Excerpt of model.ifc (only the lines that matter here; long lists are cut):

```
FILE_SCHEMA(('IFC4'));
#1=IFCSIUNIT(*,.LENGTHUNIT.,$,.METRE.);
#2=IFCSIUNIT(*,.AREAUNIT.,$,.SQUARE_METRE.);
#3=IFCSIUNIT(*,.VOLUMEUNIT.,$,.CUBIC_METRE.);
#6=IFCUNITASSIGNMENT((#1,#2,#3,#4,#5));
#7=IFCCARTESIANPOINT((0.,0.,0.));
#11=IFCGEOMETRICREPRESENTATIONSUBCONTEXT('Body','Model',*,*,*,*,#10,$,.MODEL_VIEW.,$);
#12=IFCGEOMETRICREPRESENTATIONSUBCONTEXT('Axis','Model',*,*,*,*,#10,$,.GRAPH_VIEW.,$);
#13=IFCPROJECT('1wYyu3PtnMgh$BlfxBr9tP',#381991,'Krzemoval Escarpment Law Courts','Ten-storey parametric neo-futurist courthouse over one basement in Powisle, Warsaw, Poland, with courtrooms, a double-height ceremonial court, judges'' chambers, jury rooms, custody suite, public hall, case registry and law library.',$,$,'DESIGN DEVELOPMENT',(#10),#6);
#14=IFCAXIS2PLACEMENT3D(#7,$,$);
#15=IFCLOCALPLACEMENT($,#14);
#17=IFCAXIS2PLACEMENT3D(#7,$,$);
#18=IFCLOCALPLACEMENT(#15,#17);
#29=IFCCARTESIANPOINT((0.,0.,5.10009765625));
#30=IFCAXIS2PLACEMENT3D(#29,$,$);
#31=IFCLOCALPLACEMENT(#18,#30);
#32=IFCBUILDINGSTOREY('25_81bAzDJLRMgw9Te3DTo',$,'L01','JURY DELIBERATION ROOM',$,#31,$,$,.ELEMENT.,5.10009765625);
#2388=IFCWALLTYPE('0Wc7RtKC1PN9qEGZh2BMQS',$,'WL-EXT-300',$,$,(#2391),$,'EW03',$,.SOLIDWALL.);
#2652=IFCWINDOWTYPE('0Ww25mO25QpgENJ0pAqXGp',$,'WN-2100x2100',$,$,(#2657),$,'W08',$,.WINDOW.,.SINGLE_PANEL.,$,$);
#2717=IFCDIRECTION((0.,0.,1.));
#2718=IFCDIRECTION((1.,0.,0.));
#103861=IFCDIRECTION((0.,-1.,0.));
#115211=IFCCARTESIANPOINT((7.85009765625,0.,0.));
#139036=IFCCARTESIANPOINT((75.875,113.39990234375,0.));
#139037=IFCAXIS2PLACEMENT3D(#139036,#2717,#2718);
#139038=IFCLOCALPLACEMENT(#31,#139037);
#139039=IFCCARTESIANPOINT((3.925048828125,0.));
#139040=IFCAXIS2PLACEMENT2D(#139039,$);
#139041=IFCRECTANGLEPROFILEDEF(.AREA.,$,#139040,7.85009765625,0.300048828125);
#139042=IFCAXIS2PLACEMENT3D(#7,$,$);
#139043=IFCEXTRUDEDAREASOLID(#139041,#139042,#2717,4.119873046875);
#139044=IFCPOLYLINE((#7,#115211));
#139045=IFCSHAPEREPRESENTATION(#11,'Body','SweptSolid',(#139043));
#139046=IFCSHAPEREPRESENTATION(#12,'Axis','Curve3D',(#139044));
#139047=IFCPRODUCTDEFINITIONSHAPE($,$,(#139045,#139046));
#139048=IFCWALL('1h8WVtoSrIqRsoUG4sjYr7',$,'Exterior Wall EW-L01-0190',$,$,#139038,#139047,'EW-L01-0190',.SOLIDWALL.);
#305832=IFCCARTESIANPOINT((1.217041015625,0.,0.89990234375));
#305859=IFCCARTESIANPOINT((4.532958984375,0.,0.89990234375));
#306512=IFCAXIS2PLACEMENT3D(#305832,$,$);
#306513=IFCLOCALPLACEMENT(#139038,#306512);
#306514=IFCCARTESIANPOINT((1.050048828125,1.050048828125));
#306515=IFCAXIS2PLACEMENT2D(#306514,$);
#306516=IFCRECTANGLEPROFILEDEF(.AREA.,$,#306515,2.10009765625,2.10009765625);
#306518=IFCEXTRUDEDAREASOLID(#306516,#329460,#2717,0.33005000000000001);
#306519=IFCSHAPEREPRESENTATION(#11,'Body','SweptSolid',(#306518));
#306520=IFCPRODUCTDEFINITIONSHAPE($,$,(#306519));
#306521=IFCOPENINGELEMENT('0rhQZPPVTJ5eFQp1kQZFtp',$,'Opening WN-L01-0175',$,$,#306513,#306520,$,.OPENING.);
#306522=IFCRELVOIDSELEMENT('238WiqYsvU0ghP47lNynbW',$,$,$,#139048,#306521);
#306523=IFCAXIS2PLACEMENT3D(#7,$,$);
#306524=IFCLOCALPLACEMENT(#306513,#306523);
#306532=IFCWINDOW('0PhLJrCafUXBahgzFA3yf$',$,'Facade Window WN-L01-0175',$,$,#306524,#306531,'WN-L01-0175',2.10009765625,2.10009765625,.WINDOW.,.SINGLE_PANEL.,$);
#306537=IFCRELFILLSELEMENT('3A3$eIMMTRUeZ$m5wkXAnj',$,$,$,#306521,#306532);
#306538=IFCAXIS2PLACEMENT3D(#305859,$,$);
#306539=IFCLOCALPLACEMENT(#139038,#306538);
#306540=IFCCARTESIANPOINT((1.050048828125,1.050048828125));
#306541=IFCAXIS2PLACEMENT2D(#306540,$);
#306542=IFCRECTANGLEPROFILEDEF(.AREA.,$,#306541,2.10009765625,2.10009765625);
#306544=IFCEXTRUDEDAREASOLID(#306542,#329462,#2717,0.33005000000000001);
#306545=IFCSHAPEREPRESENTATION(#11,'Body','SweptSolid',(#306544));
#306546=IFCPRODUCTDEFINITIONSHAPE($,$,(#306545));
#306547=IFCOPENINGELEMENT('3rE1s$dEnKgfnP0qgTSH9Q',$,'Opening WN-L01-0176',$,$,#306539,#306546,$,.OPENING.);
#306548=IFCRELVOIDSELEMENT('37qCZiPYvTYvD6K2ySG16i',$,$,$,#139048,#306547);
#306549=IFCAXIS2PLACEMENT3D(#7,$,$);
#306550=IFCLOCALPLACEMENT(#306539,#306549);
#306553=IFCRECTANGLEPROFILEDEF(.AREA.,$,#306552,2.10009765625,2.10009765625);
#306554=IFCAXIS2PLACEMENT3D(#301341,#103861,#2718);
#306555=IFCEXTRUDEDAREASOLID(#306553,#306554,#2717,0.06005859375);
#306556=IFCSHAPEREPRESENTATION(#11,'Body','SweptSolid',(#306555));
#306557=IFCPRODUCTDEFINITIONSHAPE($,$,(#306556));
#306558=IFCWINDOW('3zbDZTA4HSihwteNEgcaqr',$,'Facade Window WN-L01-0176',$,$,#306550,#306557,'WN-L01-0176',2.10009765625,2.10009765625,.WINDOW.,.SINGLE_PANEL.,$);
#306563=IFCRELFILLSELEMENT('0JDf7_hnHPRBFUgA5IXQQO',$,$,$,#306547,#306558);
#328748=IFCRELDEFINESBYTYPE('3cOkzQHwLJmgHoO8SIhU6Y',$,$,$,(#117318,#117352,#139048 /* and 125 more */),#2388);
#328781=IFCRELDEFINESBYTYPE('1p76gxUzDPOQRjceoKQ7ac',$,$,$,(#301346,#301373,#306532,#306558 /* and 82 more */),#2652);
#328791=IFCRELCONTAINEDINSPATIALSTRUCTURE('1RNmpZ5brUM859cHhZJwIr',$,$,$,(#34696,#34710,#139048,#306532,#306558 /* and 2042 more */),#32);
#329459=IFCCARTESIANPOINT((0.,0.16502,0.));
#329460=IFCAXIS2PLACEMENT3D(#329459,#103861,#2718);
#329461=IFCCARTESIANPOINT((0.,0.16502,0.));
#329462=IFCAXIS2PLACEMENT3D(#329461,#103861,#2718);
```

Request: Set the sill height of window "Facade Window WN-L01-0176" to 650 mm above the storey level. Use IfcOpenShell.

```python
import numpy as np
import ifcopenshell
import ifcopenshell.api.geometry
import ifcopenshell.geom
import ifcopenshell.util.element
import ifcopenshell.util.placement
import ifcopenshell.util.shape
import ifcopenshell.util.unit

model = ifcopenshell.open("model.ifc")
unit_scale = ifcopenshell.util.unit.calculate_unit_scale(model)

window = model.by_id(306558)
opening = window.FillsVoids[0].RelatingOpeningElement
storey = ifcopenshell.util.element.get_container(window, ifc_class="IfcBuildingStorey")
level = ifcopenshell.util.placement.get_local_placement(storey.ObjectPlacement)[2, 3]

# The opening's origin need not be at the sill, so measure its lowest point.
shape = ifcopenshell.geom.create_shape(ifcopenshell.geom.settings(), opening)
bottom = ifcopenshell.util.shape.get_shape_bottom_elevation(shape, shape.geometry) / unit_scale
dz = level + 0.65 / unit_scale - bottom

shift = np.array([0.0, 0.0, dz])
# The window is placed relative to its opening, so it follows when the opening moves.
matrix = ifcopenshell.util.placement.get_local_placement(opening.ObjectPlacement)
matrix[:3, 3] += shift
ifcopenshell.api.geometry.edit_object_placement(
    model, product=opening, matrix=matrix, is_si=False, should_transform_children=True
)

print(f"moved by {dz * unit_scale:+.3f} m")

model.write("model_v2.ifc")
```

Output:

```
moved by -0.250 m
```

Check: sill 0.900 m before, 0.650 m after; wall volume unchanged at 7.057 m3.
